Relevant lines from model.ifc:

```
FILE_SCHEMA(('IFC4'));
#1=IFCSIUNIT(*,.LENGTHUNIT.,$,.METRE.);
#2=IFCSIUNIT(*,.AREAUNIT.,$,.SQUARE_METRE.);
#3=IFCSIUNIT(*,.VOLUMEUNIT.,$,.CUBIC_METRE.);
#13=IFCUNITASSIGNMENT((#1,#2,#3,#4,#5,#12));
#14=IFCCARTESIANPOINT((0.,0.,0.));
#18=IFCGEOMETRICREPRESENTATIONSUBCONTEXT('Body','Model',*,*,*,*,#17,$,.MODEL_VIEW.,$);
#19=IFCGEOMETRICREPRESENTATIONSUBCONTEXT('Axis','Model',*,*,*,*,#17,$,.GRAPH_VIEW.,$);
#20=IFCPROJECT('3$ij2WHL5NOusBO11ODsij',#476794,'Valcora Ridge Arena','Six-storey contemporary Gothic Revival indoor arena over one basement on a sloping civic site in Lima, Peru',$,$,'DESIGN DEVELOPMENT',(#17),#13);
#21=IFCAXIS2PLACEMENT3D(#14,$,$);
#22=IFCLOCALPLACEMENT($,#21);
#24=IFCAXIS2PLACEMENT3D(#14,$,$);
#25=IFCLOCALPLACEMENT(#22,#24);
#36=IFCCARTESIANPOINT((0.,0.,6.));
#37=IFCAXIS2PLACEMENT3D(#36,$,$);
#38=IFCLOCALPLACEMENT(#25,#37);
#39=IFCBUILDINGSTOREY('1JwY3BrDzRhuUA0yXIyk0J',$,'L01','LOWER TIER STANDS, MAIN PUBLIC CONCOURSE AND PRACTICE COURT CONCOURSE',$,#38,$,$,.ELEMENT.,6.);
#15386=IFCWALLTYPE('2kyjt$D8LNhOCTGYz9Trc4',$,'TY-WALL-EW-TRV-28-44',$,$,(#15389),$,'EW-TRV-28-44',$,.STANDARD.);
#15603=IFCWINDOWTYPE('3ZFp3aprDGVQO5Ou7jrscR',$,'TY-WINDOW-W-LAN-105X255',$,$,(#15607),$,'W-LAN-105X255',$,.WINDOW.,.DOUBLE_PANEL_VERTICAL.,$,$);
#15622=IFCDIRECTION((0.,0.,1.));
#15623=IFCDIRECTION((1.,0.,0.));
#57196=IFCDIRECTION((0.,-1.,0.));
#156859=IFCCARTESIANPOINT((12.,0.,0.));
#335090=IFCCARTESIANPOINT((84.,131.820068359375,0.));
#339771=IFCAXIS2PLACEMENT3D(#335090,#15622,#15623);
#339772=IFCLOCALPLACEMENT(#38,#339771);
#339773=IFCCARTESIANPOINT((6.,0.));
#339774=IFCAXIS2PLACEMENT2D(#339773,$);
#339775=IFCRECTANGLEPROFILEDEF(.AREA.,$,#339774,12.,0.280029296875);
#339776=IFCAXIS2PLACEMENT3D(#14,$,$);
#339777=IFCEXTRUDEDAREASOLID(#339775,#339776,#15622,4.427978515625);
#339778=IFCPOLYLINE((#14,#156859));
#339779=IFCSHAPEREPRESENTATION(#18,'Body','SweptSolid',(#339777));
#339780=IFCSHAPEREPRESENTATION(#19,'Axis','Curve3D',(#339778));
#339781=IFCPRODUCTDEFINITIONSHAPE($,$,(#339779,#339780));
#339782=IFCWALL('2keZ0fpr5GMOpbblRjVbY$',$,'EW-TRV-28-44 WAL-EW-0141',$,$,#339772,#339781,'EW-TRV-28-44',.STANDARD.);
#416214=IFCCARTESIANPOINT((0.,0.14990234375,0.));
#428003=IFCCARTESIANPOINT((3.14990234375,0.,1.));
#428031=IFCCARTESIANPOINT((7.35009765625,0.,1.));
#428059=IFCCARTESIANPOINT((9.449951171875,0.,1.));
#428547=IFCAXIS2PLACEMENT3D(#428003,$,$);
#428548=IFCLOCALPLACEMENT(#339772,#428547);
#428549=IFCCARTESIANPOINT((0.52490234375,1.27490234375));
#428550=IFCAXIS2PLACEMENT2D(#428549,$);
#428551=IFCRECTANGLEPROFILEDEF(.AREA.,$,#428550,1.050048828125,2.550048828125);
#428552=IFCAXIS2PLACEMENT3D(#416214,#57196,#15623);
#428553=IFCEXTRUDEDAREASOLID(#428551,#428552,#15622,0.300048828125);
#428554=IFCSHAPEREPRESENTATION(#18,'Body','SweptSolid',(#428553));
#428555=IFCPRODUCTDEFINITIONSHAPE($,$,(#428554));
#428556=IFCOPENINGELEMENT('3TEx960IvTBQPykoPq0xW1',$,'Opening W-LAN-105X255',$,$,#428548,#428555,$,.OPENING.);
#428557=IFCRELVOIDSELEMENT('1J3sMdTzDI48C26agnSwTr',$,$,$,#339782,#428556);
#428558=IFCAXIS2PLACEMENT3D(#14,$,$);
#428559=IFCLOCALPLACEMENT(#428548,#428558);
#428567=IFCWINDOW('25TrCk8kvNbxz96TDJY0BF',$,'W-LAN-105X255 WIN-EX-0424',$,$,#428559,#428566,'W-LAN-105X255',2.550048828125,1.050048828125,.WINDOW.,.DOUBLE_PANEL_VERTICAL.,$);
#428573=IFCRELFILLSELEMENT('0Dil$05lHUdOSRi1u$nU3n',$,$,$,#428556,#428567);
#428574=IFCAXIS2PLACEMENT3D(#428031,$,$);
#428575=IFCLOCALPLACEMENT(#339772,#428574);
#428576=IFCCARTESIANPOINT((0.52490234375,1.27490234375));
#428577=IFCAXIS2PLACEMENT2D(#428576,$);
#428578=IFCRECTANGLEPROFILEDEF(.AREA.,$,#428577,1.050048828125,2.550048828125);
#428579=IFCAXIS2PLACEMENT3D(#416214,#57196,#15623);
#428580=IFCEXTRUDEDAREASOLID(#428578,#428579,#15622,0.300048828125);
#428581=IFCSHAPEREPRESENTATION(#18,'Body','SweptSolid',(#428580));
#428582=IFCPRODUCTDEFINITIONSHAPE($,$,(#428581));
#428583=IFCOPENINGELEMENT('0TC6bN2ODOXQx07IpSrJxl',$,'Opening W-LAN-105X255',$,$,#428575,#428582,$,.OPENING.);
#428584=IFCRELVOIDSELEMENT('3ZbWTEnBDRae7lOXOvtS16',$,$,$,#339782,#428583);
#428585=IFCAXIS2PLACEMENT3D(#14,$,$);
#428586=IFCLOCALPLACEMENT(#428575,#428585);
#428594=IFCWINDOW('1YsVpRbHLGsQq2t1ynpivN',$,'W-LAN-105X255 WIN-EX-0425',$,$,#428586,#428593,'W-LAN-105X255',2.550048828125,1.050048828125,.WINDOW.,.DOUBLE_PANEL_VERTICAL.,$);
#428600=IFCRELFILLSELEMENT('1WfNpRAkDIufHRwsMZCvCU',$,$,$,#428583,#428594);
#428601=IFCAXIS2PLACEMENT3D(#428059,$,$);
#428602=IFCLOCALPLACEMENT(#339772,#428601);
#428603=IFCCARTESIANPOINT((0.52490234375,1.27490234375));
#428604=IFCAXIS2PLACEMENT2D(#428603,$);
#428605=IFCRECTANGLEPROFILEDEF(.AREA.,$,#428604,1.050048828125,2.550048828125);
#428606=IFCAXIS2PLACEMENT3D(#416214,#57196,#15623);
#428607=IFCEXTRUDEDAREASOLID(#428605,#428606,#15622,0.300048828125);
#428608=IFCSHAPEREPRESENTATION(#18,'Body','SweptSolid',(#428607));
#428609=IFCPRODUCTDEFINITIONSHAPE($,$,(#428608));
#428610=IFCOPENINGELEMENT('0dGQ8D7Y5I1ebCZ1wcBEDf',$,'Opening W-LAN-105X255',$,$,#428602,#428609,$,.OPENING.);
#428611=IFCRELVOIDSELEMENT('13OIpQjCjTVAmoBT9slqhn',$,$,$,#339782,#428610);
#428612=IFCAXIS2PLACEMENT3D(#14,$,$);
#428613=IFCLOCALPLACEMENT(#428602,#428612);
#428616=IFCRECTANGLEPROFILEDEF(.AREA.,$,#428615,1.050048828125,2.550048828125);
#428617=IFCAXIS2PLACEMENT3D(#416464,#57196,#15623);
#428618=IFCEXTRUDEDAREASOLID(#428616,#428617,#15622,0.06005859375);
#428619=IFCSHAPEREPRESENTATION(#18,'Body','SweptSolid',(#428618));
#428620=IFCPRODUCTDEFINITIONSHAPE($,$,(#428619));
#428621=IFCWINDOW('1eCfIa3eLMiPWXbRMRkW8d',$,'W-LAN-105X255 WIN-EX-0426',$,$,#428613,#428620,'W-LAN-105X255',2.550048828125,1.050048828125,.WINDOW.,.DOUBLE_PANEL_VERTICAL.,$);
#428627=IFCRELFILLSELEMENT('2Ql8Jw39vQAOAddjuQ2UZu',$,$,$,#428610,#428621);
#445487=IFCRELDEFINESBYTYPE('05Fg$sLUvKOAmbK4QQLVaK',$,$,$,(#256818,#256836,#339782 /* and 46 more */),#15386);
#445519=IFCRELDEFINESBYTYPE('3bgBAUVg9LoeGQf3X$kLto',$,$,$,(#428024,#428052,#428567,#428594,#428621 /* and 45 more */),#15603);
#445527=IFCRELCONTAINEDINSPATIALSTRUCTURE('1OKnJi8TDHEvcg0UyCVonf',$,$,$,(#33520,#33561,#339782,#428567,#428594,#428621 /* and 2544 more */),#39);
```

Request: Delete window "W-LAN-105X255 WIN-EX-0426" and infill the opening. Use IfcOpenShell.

```python
import ifcopenshell
import ifcopenshell.api.feature
import ifcopenshell.api.root
import ifcopenshell.geom
import ifcopenshell.util.shape

model = ifcopenshell.open("model.ifc")
settings = ifcopenshell.geom.settings()


def volume(element):
    """Net volume in cubic metres, openings subtracted."""
    shape = ifcopenshell.geom.create_shape(settings, element)
    return ifcopenshell.util.shape.get_volume(shape.geometry)


window = model.by_id(428621)
opening = window.FillsVoids[0].RelatingOpeningElement
wall = opening.VoidsElements[0].RelatingBuildingElement
before = volume(wall)

ifcopenshell.api.root.remove_product(model, product=window)
ifcopenshell.api.feature.remove_feature(model, feature=opening)

after = volume(wall)

print(f"wall volume {before:.3f} -> {after:.3f} m3")

model.write("model-out.ifc")
```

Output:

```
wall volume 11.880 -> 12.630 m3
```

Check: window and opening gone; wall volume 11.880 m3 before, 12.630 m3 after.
